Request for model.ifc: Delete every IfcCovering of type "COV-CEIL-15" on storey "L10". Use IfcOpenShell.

First a look at what the model holds.

```python
import ifcopenshell
import ifcopenshell.util.element

model = ifcopenshell.open("model.ifc")
print(model.schema)
storey = next(s for s in model.by_type("IfcBuildingStorey") if s.Name == "L10")
coverings = [e for e in ifcopenshell.util.element.get_decomposition(storey) if e.is_a("IfcCovering")]
seen = {}
for e in coverings:
    element_type = ifcopenshell.util.element.get_type(e)
    name = element_type.Name if element_type not in (None, e) else None
    seen[name] = seen.get(name, 0) + 1
for name, count in sorted(seen.items(), key=str):
    print(count, "x", name)
```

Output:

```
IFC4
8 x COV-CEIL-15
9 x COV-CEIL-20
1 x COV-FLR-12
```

```python
import ifcopenshell
import ifcopenshell.api.root
import ifcopenshell.util.element

model = ifcopenshell.open("model.ifc")

storey = next(s for s in model.by_type("IfcBuildingStorey") if s.Name == "L10")
coverings = [e for e in ifcopenshell.util.element.get_decomposition(storey) if e.is_a("IfcCovering")]
targets = [e for e in coverings if (t := ifcopenshell.util.element.get_type(e)) not in (None, e) and t.Name == "COV-CEIL-15"]

for e in targets:
    ifcopenshell.api.root.remove_product(model, product=e)
print(len(targets), "removed")

model.write("model_rev.ifc")
```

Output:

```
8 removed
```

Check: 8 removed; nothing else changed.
